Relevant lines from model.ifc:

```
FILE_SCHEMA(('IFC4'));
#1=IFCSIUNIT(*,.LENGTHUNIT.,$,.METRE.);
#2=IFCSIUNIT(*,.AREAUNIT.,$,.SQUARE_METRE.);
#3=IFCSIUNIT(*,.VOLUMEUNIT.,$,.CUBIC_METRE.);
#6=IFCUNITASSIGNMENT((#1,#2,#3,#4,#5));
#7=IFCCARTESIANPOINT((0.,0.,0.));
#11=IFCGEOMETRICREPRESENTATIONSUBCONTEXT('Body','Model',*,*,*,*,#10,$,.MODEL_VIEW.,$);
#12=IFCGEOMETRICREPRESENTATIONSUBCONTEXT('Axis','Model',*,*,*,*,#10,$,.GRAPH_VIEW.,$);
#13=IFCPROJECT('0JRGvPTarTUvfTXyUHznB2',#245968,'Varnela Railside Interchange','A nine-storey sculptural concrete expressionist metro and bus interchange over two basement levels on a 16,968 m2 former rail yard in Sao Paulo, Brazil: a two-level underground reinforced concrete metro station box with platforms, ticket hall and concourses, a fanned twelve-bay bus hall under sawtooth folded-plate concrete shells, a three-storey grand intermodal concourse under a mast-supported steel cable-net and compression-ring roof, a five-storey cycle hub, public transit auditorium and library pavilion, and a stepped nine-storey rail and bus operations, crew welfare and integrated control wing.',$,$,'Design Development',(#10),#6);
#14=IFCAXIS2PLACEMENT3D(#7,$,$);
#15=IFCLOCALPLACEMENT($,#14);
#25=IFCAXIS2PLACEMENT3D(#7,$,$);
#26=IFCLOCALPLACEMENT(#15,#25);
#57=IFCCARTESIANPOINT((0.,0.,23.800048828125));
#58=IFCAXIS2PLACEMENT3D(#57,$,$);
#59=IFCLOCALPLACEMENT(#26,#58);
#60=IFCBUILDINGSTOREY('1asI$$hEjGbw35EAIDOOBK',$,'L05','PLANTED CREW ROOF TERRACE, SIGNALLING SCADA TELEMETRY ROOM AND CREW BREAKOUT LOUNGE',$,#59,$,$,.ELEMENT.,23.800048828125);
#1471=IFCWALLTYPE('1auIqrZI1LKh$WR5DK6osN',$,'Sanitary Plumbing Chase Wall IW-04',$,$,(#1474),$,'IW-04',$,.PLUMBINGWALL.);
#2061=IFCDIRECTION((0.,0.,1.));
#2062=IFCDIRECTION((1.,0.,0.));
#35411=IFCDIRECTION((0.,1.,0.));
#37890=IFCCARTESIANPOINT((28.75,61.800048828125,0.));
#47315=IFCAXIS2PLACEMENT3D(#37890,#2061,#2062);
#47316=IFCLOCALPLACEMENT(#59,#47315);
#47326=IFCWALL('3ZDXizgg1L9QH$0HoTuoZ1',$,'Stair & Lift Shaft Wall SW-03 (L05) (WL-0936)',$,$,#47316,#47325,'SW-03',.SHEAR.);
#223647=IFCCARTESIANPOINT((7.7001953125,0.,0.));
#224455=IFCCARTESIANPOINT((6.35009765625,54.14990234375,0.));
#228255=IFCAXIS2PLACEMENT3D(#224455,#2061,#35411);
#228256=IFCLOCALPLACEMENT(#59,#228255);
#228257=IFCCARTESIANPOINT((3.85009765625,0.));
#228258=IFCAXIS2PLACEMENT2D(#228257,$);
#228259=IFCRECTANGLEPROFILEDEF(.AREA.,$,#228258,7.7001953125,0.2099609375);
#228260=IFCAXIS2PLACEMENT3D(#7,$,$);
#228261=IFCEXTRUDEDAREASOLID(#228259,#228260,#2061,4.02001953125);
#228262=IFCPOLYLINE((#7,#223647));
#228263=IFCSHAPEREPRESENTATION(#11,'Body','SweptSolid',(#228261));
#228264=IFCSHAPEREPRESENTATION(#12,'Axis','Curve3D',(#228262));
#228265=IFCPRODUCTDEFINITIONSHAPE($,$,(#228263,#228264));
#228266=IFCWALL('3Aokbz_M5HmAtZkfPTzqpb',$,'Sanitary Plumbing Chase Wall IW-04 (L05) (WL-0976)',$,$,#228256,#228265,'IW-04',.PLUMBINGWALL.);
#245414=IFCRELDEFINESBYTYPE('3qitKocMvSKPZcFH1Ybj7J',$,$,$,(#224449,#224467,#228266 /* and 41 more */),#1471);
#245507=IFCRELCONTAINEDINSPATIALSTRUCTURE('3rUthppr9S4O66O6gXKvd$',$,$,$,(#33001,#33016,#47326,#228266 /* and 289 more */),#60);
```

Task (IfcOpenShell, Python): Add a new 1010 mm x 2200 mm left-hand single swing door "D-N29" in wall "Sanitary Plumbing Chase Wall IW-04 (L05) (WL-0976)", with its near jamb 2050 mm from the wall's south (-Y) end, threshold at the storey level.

```python
import numpy as np
import ifcopenshell
import ifcopenshell.api.feature
import ifcopenshell.api.geometry
import ifcopenshell.api.root
import ifcopenshell.api.spatial
import ifcopenshell.geom
import ifcopenshell.util.element
import ifcopenshell.util.placement
import ifcopenshell.util.representation
import ifcopenshell.util.shape
import ifcopenshell.util.unit

model = ifcopenshell.open("model.ifc")
unit_scale = ifcopenshell.util.unit.calculate_unit_scale(model)
settings = ifcopenshell.geom.settings()


def volume(element):
    """Net volume in cubic metres, openings subtracted."""
    shape = ifcopenshell.geom.create_shape(settings, element)
    return ifcopenshell.util.shape.get_volume(shape.geometry)


wall = model.by_guid("3Aokbz_M5HmAtZkfPTzqpb")
storey = ifcopenshell.util.element.get_container(wall, ifc_class="IfcBuildingStorey")
context = ifcopenshell.util.representation.get_context(model, "Model", "Body", "MODEL_VIEW")
before = volume(wall)

width, height, from_end, sill = 1.01, 2.2, 2.05, 0.0  # metres

# The wall runs along its own X axis, and the end named is its -X end.
wall_shape = ifcopenshell.geom.create_shape(settings, wall)
x, y, z = ifcopenshell.util.shape.get_vertices(wall_shape.geometry).T
start = x.min() + from_end
face, thickness = float(y.min()), float(y.max() - y.min())
wall_matrix = ifcopenshell.util.placement.get_local_placement(wall.ObjectPlacement)
level = ifcopenshell.util.placement.get_local_placement(storey.ObjectPlacement)[2, 3]


def in_wall(x, y):
    """Placement at x, y metres in the wall's axes, at sill height."""
    matrix = wall_matrix.copy()
    matrix[:, 3] = wall_matrix @ np.array([x / unit_scale, y / unit_scale, 0.0, 1.0])
    matrix[2, 3] = level + sill / unit_scale
    return matrix


# Opening: a box that overshoots both wall faces by 50 mm.
opening = ifcopenshell.api.root.create_entity(model, ifc_class="IfcOpeningElement", predefined_type="OPENING")
box = ifcopenshell.api.geometry.add_wall_representation(
    model, context=context, length=width, height=height, thickness=thickness + 0.1
)
ifcopenshell.api.geometry.assign_representation(model, product=opening, representation=box)
ifcopenshell.api.geometry.edit_object_placement(model, product=opening, matrix=in_wall(start, face - 0.05), is_si=False)
ifcopenshell.api.feature.add_feature(model, feature=opening, element=wall)

door = ifcopenshell.api.root.create_entity(model, ifc_class="IfcDoor", name="D-N29", predefined_type="DOOR")
door.OverallWidth, door.OverallHeight = width / unit_scale, height / unit_scale
door.OperationType = "SINGLE_SWING_LEFT"
body = ifcopenshell.api.geometry.add_door_representation(
    model,
    context=context,
    overall_width=door.OverallWidth,
    overall_height=door.OverallHeight,
    operation_type="SINGLE_SWING_LEFT",
    lining_properties={"LiningDepth": thickness / unit_scale, "ThresholdDepth": thickness / unit_scale},
)
ifcopenshell.api.geometry.assign_representation(model, product=door, representation=body)
ifcopenshell.api.spatial.assign_container(model, products=[door], relating_structure=storey)
ifcopenshell.api.feature.add_filling(model, opening=opening, element=door)

# The lining spans the wall, so the door starts at the wall face.
ifcopenshell.api.geometry.edit_object_placement(model, product=door, matrix=in_wall(start, face), is_si=False)

after = volume(wall)

print(f"wall volume {before:.3f} -> {after:.3f} m3")

model.write("model_rev.ifc")
```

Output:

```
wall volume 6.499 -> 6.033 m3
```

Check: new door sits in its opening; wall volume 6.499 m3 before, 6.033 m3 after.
